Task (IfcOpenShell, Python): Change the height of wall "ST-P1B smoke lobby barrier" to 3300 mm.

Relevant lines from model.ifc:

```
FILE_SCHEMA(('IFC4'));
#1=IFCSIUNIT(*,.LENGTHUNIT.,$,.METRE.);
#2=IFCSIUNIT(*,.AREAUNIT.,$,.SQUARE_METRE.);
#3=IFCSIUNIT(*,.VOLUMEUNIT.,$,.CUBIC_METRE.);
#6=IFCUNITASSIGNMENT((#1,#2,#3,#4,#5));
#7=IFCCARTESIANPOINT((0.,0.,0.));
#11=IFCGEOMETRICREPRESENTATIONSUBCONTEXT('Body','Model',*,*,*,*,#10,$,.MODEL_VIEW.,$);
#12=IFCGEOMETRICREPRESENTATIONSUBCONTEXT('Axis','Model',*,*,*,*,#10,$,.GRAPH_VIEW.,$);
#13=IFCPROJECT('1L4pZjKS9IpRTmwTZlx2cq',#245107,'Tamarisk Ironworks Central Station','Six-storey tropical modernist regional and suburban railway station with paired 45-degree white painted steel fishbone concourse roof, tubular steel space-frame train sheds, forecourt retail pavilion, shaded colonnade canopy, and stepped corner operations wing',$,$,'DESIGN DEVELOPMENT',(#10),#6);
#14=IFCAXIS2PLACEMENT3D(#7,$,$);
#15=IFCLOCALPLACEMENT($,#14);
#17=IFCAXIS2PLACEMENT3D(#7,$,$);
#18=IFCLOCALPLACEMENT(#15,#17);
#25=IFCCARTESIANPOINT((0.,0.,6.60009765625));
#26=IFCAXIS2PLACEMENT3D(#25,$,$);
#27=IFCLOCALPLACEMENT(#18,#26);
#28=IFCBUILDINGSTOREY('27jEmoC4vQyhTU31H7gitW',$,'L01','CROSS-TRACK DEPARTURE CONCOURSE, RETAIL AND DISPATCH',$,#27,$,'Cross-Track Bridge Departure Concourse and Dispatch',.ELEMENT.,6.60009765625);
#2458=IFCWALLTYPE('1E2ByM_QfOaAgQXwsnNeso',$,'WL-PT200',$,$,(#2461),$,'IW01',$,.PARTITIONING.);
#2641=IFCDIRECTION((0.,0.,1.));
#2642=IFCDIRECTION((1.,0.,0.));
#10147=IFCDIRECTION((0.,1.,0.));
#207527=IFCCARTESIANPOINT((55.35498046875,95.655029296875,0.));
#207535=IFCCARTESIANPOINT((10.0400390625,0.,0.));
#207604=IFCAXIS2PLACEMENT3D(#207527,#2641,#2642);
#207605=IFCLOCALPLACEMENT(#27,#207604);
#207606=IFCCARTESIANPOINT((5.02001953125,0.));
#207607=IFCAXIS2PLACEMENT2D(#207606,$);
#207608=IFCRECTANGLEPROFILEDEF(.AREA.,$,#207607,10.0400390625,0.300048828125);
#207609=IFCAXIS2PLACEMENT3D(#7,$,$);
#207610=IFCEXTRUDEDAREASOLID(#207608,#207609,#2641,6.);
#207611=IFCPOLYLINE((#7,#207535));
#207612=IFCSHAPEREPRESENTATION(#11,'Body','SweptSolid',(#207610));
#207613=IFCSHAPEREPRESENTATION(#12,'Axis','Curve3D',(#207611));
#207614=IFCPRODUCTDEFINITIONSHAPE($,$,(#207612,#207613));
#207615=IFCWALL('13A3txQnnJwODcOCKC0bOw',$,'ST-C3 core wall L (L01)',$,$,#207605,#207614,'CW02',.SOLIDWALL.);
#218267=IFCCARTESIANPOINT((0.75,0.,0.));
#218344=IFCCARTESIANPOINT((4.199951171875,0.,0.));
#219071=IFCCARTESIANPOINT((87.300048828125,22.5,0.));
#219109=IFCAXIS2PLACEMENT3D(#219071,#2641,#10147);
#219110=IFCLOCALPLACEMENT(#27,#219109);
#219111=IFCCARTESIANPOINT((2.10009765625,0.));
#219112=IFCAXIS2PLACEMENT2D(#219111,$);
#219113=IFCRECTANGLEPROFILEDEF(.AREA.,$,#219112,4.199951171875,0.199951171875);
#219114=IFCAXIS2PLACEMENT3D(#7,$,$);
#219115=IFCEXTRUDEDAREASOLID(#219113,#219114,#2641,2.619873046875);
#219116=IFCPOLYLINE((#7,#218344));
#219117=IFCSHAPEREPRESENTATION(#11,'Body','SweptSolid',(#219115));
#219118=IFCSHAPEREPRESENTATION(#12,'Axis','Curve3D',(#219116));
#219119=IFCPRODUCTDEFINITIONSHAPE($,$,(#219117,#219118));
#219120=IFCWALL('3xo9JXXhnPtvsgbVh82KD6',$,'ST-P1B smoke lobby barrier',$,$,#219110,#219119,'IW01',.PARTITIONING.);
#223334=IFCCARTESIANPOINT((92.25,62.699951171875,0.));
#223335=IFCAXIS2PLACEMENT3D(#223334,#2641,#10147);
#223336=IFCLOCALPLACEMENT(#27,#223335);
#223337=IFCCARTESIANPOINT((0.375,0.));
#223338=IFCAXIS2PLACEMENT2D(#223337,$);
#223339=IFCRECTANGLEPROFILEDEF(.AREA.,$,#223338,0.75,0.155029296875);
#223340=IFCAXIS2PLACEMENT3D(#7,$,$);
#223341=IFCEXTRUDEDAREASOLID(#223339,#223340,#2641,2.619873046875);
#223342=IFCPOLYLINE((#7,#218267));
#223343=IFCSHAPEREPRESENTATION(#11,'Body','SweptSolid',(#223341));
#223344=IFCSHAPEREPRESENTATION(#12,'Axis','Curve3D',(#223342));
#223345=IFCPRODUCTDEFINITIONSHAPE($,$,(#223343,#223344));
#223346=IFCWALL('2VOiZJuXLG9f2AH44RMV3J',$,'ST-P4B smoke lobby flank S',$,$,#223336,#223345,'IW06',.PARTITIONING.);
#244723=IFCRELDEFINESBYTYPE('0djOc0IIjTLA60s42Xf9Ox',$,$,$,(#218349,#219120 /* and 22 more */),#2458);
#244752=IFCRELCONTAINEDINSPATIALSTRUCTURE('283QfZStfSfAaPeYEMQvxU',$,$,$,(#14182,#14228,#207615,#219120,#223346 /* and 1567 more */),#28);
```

```python
import ifcopenshell
import ifcopenshell.geom
import ifcopenshell.util.representation
import ifcopenshell.util.shape
import ifcopenshell.util.unit

model = ifcopenshell.open("model.ifc")
unit_scale = ifcopenshell.util.unit.calculate_unit_scale(model)
settings = ifcopenshell.geom.settings()


def volume(element):
    """Net volume in cubic metres, openings subtracted."""
    shape = ifcopenshell.geom.create_shape(settings, element)
    return ifcopenshell.util.shape.get_volume(shape.geometry)


wall = model.by_guid("3xo9JXXhnPtvsgbVh82KD6")
before = volume(wall)

body = ifcopenshell.util.representation.get_representation(wall, "Model", "Body")
solid = body.Items[0]
old_height = solid.Depth
solid.Depth = 3.3 / unit_scale
after = volume(wall)

print(f"height {old_height:g} -> {solid.Depth:g}, volume {before:.3f} -> {after:.3f} m3")

model.write("model_v2.ifc")
```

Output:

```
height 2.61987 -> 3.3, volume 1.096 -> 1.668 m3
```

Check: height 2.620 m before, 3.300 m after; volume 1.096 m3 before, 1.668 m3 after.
